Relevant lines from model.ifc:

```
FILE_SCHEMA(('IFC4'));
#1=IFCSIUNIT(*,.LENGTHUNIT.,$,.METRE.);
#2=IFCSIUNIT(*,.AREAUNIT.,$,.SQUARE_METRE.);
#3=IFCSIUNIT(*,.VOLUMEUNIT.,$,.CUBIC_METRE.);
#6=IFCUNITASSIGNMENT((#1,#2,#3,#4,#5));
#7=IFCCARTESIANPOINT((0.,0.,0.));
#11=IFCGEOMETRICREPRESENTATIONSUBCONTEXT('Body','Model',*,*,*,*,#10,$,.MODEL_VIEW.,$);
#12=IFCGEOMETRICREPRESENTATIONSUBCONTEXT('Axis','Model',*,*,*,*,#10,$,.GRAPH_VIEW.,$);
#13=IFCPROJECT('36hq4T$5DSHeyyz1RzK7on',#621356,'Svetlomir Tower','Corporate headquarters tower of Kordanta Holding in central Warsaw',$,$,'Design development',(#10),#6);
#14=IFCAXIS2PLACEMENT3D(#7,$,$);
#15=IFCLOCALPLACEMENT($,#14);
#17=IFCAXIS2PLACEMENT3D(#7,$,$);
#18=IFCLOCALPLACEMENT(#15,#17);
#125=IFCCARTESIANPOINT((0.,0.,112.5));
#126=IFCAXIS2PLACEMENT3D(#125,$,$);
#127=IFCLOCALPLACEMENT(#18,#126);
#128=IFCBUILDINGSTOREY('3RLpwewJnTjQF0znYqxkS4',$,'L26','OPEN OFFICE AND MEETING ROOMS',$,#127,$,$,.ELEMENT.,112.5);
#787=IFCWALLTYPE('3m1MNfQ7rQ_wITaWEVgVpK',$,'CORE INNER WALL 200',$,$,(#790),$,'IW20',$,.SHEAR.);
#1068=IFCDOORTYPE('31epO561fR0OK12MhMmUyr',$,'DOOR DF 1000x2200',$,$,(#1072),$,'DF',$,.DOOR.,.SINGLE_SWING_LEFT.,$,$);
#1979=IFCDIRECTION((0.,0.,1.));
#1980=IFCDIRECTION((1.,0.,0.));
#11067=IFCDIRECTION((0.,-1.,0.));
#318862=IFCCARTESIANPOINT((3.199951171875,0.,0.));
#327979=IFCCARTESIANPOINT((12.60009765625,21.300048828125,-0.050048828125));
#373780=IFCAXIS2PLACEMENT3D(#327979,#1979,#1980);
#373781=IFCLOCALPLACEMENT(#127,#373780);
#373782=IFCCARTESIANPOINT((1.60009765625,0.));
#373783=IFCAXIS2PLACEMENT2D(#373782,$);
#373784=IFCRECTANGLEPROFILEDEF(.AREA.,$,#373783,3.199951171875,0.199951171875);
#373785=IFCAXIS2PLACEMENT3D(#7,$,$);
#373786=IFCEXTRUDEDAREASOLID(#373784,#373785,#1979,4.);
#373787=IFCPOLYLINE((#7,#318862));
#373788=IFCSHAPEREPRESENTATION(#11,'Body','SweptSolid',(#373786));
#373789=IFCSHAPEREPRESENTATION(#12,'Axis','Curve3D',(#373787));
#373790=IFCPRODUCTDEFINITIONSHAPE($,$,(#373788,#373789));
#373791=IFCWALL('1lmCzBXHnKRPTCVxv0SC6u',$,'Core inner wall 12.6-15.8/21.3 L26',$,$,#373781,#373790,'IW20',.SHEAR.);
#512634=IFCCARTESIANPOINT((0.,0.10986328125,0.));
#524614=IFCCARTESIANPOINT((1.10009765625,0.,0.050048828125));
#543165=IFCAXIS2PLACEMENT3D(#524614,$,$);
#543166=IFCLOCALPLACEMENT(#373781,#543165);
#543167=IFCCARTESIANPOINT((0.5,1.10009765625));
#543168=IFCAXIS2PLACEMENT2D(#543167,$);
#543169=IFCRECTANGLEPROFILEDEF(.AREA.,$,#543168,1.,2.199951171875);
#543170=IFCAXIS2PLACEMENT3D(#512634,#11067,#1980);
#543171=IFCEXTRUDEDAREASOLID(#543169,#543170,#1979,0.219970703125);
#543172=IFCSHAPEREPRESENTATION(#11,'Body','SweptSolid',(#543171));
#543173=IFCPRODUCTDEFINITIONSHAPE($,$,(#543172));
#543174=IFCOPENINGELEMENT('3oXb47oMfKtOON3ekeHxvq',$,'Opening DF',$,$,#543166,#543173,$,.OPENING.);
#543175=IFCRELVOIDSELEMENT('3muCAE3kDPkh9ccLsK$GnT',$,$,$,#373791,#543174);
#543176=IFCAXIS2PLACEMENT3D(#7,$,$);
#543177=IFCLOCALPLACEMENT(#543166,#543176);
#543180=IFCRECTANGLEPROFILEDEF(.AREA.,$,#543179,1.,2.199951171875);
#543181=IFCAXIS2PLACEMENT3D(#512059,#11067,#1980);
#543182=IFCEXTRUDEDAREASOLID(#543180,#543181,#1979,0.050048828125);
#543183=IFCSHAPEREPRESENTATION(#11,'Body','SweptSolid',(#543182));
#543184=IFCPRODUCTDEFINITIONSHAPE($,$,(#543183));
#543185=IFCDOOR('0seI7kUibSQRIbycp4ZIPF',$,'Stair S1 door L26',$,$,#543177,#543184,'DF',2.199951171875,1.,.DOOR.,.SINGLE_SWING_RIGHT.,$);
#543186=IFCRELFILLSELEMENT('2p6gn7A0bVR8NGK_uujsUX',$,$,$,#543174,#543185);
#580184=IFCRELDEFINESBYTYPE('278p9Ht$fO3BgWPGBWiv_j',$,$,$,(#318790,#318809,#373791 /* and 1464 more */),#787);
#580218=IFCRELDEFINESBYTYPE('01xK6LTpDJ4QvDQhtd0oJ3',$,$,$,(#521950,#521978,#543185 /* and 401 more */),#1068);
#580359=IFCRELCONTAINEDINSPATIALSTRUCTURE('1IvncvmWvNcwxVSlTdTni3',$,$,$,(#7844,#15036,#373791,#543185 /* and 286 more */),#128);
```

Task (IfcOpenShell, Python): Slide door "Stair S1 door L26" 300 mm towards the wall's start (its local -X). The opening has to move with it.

```python
import ifcopenshell
import ifcopenshell.api.geometry
import ifcopenshell.util.placement
import ifcopenshell.util.unit

model = ifcopenshell.open("model.ifc")
unit_scale = ifcopenshell.util.unit.calculate_unit_scale(model)

door = model.by_guid("0seI7kUibSQRIbycp4ZIPF")
opening = door.FillsVoids[0].RelatingOpeningElement
wall = opening.VoidsElements[0].RelatingBuildingElement

wall_matrix = ifcopenshell.util.placement.get_local_placement(wall.ObjectPlacement)
shift = wall_matrix[:3, 0] * -0.3 / unit_scale
before = ifcopenshell.util.placement.get_local_placement(door.ObjectPlacement)[:3, 3].copy()

# The door is placed relative to its opening, so it follows when the opening moves.
matrix = ifcopenshell.util.placement.get_local_placement(opening.ObjectPlacement)
matrix[:3, 3] += shift
ifcopenshell.api.geometry.edit_object_placement(
    model, product=opening, matrix=matrix, is_si=False, should_transform_children=True
)

after = ifcopenshell.util.placement.get_local_placement(door.ObjectPlacement)[:3, 3]
print("door moved by", (after - before).round(3) + 0.0)

model.write("model_rev.ifc")
```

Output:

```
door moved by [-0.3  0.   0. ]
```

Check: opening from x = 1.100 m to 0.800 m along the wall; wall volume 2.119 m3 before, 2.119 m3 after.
